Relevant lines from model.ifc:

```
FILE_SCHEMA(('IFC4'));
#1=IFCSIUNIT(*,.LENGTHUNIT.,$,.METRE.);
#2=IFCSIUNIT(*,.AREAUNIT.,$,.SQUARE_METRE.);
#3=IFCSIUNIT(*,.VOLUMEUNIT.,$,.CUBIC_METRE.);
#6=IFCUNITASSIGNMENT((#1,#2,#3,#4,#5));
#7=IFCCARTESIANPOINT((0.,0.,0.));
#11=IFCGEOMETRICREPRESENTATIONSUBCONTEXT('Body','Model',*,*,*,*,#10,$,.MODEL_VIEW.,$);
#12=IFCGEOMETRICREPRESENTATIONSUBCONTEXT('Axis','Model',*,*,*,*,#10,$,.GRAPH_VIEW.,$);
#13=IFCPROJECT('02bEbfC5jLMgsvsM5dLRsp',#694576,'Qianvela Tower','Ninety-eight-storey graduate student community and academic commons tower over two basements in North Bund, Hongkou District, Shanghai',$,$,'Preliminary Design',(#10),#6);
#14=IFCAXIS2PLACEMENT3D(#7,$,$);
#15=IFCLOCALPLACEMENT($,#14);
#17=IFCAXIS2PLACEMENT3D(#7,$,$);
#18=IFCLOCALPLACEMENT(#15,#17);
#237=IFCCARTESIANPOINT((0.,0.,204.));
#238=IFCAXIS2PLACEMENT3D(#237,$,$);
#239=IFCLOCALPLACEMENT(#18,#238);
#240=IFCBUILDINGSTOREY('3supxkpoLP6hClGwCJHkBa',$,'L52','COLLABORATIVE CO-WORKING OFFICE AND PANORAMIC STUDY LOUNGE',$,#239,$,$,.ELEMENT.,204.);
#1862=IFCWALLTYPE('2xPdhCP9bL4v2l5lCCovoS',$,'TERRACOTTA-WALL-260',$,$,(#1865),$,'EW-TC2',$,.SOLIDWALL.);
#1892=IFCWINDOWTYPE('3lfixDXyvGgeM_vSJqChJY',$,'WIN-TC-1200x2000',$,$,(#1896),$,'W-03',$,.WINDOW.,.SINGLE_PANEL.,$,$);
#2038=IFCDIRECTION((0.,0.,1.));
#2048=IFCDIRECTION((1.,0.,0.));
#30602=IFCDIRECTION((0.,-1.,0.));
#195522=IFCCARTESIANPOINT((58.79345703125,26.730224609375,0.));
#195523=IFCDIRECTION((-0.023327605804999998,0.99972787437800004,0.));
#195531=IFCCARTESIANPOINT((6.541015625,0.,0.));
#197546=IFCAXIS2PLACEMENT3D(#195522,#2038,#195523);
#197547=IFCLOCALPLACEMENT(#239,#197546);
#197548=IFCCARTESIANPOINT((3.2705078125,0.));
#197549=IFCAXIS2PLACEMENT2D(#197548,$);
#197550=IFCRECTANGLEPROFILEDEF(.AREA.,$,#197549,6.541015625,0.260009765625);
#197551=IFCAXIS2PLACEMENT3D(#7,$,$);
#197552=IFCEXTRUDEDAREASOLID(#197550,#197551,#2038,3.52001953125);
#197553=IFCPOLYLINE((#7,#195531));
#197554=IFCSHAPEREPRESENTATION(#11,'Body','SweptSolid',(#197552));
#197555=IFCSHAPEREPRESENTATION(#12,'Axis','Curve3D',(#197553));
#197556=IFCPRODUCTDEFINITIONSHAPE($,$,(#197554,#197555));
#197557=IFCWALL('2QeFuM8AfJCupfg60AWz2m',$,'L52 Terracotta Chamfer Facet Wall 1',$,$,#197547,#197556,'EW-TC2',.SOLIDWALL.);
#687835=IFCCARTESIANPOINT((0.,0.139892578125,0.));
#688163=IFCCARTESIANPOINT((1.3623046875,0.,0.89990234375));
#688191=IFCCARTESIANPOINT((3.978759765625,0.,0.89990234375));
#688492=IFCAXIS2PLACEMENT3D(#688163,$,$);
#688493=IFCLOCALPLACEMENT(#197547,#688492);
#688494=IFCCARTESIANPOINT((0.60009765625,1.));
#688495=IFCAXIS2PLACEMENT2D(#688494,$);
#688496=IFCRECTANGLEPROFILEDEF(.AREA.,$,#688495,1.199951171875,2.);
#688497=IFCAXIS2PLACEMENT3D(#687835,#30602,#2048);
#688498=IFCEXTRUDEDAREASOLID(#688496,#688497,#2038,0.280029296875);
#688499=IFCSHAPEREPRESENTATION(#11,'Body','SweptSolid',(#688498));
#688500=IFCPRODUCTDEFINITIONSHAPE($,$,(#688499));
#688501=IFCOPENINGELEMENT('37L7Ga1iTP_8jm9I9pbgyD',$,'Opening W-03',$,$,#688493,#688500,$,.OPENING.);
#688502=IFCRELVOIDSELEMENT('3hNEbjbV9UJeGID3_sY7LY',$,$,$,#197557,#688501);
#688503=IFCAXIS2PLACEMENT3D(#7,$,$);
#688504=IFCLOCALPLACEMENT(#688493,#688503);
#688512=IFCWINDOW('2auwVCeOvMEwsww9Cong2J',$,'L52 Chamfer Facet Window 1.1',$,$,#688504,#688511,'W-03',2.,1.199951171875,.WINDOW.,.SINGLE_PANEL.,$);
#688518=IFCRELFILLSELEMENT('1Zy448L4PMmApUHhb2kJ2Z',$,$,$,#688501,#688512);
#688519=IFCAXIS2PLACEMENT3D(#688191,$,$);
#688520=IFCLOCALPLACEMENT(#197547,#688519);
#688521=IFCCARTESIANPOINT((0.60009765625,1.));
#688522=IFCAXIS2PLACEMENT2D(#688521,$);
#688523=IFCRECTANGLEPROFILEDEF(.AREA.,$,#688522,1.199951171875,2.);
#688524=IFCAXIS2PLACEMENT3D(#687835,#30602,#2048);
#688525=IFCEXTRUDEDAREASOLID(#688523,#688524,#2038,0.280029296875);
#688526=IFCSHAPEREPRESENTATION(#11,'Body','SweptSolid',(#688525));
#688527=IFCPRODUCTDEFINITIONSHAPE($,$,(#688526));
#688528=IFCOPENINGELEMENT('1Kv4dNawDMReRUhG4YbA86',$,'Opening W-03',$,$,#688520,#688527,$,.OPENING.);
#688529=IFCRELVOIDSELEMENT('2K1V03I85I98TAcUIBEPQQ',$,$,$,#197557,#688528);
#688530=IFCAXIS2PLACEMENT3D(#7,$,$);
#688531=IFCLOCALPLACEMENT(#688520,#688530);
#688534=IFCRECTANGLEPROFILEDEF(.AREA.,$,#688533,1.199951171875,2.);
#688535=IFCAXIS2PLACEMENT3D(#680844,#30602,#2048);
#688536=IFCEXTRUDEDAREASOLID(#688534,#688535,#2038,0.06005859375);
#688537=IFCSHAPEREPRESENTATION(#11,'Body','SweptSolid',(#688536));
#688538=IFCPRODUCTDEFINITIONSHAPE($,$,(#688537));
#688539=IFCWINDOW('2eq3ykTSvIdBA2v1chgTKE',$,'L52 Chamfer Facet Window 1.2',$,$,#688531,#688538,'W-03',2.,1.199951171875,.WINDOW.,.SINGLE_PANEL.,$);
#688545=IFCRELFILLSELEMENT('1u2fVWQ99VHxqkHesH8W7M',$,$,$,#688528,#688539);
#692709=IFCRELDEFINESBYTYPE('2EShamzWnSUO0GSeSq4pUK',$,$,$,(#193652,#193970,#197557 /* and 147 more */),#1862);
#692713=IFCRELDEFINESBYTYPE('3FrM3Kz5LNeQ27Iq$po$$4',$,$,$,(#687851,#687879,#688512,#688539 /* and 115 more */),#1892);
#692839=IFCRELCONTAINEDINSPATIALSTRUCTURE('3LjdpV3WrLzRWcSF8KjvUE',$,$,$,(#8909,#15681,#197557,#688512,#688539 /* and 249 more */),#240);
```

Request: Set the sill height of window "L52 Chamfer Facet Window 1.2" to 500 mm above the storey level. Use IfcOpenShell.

```python
import numpy as np
import ifcopenshell
import ifcopenshell.api.geometry
import ifcopenshell.geom
import ifcopenshell.util.element
import ifcopenshell.util.placement
import ifcopenshell.util.shape
import ifcopenshell.util.unit

model = ifcopenshell.open("model.ifc")
unit_scale = ifcopenshell.util.unit.calculate_unit_scale(model)

window = model.by_guid("2eq3ykTSvIdBA2v1chgTKE")
opening = window.FillsVoids[0].RelatingOpeningElement
storey = ifcopenshell.util.element.get_container(window, ifc_class="IfcBuildingStorey")
level = ifcopenshell.util.placement.get_local_placement(storey.ObjectPlacement)[2, 3]

# The opening's origin need not be at the sill, so measure its lowest point.
shape = ifcopenshell.geom.create_shape(ifcopenshell.geom.settings(), opening)
bottom = ifcopenshell.util.shape.get_shape_bottom_elevation(shape, shape.geometry) / unit_scale
dz = level + 0.5 - bottom

shift = np.array([0.0, 0.0, dz])
# The window is placed relative to its opening, so it follows when the opening moves.
matrix = ifcopenshell.util.placement.get_local_placement(opening.ObjectPlacement)
matrix[:3, 3] += shift
ifcopenshell.api.geometry.edit_object_placement(
    model, product=opening, matrix=matrix, is_si=False, should_transform_children=True
)

print(f"moved by {dz * unit_scale:+.3f} m")

model.write("model_v2.ifc")
```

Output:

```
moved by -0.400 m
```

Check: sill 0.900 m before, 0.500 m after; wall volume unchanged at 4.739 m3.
